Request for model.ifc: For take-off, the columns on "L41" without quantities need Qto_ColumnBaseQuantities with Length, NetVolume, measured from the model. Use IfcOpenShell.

First a look at what the model holds.

```python
import ifcopenshell
import ifcopenshell.util.element
import ifcopenshell.util.unit

model = ifcopenshell.open("model.ifc")
print(model.schema)
for unit_type in ("LENGTHUNIT", "AREAUNIT", "VOLUMEUNIT"):
    print(unit_type, ifcopenshell.util.unit.calculate_unit_scale(model, unit_type))
storey = next(s for s in model.by_type("IfcBuildingStorey") if s.Name == "L41")
columns = [e for e in ifcopenshell.util.element.get_decomposition(storey) if e.is_a("IfcColumn")]
for e in sorted(columns, key=lambda e: e.id()):
    print(e.id(), e.is_a(), e.Name, list(ifcopenshell.util.element.get_psets(e, qtos_only=True)), sep=" | ")
```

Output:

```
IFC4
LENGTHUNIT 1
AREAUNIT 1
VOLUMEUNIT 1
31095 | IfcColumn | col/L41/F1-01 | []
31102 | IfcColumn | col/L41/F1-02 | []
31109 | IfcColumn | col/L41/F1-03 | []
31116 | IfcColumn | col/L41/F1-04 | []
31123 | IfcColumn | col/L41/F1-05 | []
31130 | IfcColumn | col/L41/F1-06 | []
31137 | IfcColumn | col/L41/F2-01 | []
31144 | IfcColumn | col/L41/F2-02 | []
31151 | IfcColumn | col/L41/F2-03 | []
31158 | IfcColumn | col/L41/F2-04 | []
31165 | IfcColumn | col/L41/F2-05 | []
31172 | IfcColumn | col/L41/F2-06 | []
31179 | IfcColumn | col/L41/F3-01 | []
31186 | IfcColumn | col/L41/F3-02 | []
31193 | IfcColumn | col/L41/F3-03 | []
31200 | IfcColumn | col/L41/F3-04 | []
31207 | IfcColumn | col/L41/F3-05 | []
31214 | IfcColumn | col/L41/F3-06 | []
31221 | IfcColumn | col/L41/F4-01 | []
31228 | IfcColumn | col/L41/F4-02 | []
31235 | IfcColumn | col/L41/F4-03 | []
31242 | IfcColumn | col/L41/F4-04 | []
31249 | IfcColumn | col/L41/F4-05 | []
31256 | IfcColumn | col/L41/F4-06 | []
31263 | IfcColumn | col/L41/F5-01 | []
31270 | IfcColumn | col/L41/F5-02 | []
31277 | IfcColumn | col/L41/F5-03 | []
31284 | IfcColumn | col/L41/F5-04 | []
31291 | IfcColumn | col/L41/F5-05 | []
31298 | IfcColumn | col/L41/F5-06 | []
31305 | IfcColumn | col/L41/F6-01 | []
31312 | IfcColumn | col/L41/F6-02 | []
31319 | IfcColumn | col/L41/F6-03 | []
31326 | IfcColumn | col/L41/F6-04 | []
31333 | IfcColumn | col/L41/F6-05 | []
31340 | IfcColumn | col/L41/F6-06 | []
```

```python
import ifcopenshell
import ifcopenshell.api.pset
import ifcopenshell.geom
import ifcopenshell.util.element
import ifcopenshell.util.shape
import ifcopenshell.util.unit

model = ifcopenshell.open("model.ifc")
unit_scale = ifcopenshell.util.unit.calculate_unit_scale(model)
volume_scale = ifcopenshell.util.unit.calculate_unit_scale(model, "VOLUMEUNIT")
settings = ifcopenshell.geom.settings()

storey = next(s for s in model.by_type("IfcBuildingStorey") if s.Name == "L41")
columns = [e for e in ifcopenshell.util.element.get_decomposition(storey) if e.is_a("IfcColumn")]

for e in sorted(columns, key=lambda e: e.id()):
    if ifcopenshell.util.element.get_psets(e, qtos_only=True, should_inherit=False):
        continue
    # Geometry comes back in metres, in the element's own axes.
    shape = ifcopenshell.geom.create_shape(settings, e)
    values = {
        "Length": ifcopenshell.util.shape.get_z(shape.geometry) / unit_scale,
        "NetVolume": ifcopenshell.util.shape.get_volume(shape.geometry) / volume_scale,
    }
    qto = ifcopenshell.api.pset.add_qto(model, product=e, name="Qto_ColumnBaseQuantities")
    ifcopenshell.api.pset.edit_qto(model, qto=qto, properties=values)
    print(e.id(), {k: round(v, 3) for k, v in values.items()})

model.write("model-out.ifc")
```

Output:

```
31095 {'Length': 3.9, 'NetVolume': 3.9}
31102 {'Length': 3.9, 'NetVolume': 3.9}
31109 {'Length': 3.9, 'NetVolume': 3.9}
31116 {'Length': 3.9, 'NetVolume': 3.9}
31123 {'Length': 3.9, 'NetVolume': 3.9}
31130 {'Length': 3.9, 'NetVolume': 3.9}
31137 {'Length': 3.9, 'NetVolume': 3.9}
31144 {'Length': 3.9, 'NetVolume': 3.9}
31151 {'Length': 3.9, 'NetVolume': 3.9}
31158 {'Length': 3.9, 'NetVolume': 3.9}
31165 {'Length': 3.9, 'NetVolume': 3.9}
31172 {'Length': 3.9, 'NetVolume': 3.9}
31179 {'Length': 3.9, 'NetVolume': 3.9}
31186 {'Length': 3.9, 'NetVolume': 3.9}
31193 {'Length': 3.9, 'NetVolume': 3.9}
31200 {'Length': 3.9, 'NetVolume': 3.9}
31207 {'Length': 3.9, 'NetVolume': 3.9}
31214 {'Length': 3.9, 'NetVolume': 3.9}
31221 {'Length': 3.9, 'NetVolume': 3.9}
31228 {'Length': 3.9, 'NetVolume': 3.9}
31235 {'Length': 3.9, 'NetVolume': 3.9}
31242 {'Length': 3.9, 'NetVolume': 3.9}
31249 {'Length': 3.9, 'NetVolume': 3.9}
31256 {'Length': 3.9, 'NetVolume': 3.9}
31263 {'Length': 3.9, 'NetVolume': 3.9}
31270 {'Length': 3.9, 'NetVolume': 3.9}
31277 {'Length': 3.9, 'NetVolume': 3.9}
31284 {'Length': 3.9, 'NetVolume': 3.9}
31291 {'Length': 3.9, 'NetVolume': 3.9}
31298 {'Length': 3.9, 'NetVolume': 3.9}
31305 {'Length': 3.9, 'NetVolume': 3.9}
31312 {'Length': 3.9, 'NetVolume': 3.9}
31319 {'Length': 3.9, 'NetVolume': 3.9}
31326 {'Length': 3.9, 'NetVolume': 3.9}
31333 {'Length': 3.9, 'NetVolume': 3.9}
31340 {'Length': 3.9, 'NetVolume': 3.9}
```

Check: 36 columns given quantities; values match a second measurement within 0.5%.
